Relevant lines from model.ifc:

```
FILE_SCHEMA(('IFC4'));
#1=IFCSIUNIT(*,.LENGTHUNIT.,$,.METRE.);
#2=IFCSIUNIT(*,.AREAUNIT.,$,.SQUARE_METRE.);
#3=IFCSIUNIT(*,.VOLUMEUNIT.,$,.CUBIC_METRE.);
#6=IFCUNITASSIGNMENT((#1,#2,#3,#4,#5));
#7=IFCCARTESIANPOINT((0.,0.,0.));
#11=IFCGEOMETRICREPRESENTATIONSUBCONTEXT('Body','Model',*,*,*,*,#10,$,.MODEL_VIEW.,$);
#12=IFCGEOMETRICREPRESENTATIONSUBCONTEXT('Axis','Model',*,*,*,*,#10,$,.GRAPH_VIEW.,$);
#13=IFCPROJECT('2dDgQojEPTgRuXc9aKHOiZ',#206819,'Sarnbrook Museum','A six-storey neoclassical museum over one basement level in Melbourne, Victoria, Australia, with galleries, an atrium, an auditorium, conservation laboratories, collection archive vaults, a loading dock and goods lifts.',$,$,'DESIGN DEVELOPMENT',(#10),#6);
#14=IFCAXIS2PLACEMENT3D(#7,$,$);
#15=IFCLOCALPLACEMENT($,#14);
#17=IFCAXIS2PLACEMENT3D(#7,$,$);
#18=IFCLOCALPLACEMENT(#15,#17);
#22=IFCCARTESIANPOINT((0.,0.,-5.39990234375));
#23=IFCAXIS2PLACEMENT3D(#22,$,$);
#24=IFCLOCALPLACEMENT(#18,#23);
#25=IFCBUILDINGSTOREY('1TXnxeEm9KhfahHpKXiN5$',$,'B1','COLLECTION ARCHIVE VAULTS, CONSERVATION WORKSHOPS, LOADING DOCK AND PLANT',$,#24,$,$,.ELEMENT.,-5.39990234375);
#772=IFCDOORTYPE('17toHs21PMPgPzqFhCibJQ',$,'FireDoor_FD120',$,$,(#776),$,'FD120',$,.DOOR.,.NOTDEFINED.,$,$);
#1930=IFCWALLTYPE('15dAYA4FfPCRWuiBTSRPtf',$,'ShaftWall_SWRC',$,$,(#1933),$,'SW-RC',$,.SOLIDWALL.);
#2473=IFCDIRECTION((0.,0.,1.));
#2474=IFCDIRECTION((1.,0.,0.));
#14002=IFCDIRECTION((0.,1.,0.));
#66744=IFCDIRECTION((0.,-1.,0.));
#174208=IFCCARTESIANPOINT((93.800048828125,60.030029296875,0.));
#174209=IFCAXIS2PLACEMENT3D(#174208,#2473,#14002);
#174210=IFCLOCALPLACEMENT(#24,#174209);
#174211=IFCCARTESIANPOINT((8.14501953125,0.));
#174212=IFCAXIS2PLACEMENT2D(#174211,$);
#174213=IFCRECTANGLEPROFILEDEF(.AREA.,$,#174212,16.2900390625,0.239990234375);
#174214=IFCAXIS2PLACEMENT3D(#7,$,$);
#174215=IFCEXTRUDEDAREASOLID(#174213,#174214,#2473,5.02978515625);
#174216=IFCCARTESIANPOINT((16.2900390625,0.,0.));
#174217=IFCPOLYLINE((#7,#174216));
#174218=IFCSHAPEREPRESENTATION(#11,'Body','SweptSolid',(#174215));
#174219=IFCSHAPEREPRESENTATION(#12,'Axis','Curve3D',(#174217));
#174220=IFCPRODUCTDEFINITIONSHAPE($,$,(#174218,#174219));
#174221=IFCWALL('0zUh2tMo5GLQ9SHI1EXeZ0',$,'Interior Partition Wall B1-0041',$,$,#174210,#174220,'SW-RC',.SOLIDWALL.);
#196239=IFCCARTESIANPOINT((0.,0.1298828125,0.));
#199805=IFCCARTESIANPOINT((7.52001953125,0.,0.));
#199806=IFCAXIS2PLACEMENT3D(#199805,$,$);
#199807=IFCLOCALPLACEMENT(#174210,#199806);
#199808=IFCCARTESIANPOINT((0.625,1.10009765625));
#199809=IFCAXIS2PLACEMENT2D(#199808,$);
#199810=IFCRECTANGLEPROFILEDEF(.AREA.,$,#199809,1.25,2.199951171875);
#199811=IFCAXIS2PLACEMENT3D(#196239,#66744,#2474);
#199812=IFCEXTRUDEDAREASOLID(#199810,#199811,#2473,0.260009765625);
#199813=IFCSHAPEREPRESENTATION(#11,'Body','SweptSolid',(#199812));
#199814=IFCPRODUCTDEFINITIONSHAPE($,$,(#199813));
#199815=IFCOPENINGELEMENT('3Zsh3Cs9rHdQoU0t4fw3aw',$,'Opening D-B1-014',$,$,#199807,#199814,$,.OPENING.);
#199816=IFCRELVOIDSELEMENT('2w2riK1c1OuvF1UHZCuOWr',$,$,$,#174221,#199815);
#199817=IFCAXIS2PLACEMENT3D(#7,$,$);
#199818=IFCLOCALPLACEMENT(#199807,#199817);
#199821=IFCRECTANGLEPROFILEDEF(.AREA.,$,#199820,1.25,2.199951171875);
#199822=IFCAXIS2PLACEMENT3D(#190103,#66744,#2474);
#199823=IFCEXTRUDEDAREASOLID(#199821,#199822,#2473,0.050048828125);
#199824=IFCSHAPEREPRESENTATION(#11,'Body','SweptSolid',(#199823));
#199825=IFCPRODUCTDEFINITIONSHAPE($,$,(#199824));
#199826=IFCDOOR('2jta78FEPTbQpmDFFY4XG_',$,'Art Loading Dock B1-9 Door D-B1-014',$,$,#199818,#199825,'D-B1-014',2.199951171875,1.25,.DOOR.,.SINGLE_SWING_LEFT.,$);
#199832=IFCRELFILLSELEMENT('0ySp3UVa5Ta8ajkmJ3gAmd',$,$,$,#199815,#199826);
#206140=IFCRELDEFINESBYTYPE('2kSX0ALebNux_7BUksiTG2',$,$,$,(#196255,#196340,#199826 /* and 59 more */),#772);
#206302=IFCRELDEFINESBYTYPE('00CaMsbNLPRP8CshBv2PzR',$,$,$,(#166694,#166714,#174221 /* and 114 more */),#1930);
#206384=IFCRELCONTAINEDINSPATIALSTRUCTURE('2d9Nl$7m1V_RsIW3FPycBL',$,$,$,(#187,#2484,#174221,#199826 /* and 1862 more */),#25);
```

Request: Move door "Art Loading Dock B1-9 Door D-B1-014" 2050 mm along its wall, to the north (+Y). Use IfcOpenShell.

```python
import ifcopenshell
import ifcopenshell.api.geometry
import ifcopenshell.util.placement

model = ifcopenshell.open("model.ifc")

door = model.by_guid("2jta78FEPTbQpmDFFY4XG_")
opening = door.FillsVoids[0].RelatingOpeningElement
wall = opening.VoidsElements[0].RelatingBuildingElement

wall_matrix = ifcopenshell.util.placement.get_local_placement(wall.ObjectPlacement)
shift = wall_matrix[:3, 0] * 2.05
before = ifcopenshell.util.placement.get_local_placement(door.ObjectPlacement)[:3, 3].copy()

# The door is placed relative to its opening, so it follows when the opening moves.
matrix = ifcopenshell.util.placement.get_local_placement(opening.ObjectPlacement)
matrix[:3, 3] += shift
ifcopenshell.api.geometry.edit_object_placement(
    model, product=opening, matrix=matrix, is_si=False, should_transform_children=True
)

after = ifcopenshell.util.placement.get_local_placement(door.ObjectPlacement)[:3, 3]
print("door moved by", (after - before).round(3) + 0.0)

model.write("model_updated.ifc")
```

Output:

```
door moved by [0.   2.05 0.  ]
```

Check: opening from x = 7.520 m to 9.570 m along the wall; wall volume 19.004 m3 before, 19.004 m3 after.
